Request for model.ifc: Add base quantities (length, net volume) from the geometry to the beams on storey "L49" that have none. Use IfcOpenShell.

First a look at what the model holds.

```python
import ifcopenshell
import ifcopenshell.util.element
import ifcopenshell.util.unit

model = ifcopenshell.open("model.ifc")
print(model.schema)
for unit_type in ("LENGTHUNIT", "AREAUNIT", "VOLUMEUNIT"):
    print(unit_type, ifcopenshell.util.unit.calculate_unit_scale(model, unit_type))
storey = next(s for s in model.by_type("IfcBuildingStorey") if s.Name == "L49")
beams = [e for e in ifcopenshell.util.element.get_decomposition(storey) if e.is_a("IfcBeam")]
for e in sorted(beams, key=lambda e: e.id()):
    print(e.id(), e.is_a(), e.Name, list(ifcopenshell.util.element.get_psets(e, qtos_only=True)), sep=" | ")
```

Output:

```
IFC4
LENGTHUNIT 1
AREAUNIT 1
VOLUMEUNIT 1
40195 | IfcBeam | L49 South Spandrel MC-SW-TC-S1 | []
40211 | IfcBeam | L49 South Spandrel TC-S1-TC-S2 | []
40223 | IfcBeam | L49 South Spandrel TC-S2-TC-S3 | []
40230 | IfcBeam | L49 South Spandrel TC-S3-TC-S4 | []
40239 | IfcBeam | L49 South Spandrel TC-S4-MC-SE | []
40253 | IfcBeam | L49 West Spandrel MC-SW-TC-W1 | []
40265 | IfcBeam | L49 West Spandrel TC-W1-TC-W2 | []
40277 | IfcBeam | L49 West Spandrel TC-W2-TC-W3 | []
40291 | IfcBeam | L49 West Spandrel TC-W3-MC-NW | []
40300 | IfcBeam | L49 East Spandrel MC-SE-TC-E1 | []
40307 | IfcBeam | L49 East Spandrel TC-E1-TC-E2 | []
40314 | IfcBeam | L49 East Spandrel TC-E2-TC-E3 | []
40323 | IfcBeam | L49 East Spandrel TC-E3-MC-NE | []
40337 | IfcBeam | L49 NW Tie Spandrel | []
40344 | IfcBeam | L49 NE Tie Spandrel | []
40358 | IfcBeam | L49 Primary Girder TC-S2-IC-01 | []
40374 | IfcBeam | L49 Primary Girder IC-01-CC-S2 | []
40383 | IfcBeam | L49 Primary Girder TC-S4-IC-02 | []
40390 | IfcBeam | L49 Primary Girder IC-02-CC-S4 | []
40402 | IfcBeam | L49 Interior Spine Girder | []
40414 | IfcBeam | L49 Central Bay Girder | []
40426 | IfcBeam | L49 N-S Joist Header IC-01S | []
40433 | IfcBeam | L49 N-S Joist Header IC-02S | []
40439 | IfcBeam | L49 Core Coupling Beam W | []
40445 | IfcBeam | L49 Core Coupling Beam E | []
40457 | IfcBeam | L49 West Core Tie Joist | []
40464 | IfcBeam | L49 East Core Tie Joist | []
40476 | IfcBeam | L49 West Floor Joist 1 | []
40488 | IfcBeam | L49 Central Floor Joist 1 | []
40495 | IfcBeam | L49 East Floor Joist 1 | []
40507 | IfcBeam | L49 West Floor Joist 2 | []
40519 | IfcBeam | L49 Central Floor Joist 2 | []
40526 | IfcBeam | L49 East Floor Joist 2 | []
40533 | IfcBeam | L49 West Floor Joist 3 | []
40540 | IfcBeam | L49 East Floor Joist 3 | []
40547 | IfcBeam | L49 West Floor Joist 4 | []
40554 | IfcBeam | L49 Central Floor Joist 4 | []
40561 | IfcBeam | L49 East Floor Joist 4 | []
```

```python
import ifcopenshell
import ifcopenshell.api.pset
import ifcopenshell.geom
import ifcopenshell.util.element
import ifcopenshell.util.shape
import ifcopenshell.util.unit

model = ifcopenshell.open("model.ifc")
unit_scale = ifcopenshell.util.unit.calculate_unit_scale(model)
volume_scale = ifcopenshell.util.unit.calculate_unit_scale(model, "VOLUMEUNIT")
settings = ifcopenshell.geom.settings()

storey = next(s for s in model.by_type("IfcBuildingStorey") if s.Name == "L49")
beams = [e for e in ifcopenshell.util.element.get_decomposition(storey) if e.is_a("IfcBeam")]

for e in sorted(beams, key=lambda e: e.id()):
    if ifcopenshell.util.element.get_psets(e, qtos_only=True, should_inherit=False):
        continue
    # Geometry comes back in metres, in the element's own axes.
    shape = ifcopenshell.geom.create_shape(settings, e)
    values = {
        "Length": ifcopenshell.util.shape.get_max_xyz(shape.geometry) / unit_scale,
        "NetVolume": ifcopenshell.util.shape.get_volume(shape.geometry) / volume_scale,
    }
    qto = ifcopenshell.api.pset.add_qto(model, product=e, name="Qto_BeamBaseQuantities")
    ifcopenshell.api.pset.edit_qto(model, qto=qto, properties=values)
    print(e.id(), {k: round(v, 3) for k, v in values.items()})

model.write("model_v2.ifc")
```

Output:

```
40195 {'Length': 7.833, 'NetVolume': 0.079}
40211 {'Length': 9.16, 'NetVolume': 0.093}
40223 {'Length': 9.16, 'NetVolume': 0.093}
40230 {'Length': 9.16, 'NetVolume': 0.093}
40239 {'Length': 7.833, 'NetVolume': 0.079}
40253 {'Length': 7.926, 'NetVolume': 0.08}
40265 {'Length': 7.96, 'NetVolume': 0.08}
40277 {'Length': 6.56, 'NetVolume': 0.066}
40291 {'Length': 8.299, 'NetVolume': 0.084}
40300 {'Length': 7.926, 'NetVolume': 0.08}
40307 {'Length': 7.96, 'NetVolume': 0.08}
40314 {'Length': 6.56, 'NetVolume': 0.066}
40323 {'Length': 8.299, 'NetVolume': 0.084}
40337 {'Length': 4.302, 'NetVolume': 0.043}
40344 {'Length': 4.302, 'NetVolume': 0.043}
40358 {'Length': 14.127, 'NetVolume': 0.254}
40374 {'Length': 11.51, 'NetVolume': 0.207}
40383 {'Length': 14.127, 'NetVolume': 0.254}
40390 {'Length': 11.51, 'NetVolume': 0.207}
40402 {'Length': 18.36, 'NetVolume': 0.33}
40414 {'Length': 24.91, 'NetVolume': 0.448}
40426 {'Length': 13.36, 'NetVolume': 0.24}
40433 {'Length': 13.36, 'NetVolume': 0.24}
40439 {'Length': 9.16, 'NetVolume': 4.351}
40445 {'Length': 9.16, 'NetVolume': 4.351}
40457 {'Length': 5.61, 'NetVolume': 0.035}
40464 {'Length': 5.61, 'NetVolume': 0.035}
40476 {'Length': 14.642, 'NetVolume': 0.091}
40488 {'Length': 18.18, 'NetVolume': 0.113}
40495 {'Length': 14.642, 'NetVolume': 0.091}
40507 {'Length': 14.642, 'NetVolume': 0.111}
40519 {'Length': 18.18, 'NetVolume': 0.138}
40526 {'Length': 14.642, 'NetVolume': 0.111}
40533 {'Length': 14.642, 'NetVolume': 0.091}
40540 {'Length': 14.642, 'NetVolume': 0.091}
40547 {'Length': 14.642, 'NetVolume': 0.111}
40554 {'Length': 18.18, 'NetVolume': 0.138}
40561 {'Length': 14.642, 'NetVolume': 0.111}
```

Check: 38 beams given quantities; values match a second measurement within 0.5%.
